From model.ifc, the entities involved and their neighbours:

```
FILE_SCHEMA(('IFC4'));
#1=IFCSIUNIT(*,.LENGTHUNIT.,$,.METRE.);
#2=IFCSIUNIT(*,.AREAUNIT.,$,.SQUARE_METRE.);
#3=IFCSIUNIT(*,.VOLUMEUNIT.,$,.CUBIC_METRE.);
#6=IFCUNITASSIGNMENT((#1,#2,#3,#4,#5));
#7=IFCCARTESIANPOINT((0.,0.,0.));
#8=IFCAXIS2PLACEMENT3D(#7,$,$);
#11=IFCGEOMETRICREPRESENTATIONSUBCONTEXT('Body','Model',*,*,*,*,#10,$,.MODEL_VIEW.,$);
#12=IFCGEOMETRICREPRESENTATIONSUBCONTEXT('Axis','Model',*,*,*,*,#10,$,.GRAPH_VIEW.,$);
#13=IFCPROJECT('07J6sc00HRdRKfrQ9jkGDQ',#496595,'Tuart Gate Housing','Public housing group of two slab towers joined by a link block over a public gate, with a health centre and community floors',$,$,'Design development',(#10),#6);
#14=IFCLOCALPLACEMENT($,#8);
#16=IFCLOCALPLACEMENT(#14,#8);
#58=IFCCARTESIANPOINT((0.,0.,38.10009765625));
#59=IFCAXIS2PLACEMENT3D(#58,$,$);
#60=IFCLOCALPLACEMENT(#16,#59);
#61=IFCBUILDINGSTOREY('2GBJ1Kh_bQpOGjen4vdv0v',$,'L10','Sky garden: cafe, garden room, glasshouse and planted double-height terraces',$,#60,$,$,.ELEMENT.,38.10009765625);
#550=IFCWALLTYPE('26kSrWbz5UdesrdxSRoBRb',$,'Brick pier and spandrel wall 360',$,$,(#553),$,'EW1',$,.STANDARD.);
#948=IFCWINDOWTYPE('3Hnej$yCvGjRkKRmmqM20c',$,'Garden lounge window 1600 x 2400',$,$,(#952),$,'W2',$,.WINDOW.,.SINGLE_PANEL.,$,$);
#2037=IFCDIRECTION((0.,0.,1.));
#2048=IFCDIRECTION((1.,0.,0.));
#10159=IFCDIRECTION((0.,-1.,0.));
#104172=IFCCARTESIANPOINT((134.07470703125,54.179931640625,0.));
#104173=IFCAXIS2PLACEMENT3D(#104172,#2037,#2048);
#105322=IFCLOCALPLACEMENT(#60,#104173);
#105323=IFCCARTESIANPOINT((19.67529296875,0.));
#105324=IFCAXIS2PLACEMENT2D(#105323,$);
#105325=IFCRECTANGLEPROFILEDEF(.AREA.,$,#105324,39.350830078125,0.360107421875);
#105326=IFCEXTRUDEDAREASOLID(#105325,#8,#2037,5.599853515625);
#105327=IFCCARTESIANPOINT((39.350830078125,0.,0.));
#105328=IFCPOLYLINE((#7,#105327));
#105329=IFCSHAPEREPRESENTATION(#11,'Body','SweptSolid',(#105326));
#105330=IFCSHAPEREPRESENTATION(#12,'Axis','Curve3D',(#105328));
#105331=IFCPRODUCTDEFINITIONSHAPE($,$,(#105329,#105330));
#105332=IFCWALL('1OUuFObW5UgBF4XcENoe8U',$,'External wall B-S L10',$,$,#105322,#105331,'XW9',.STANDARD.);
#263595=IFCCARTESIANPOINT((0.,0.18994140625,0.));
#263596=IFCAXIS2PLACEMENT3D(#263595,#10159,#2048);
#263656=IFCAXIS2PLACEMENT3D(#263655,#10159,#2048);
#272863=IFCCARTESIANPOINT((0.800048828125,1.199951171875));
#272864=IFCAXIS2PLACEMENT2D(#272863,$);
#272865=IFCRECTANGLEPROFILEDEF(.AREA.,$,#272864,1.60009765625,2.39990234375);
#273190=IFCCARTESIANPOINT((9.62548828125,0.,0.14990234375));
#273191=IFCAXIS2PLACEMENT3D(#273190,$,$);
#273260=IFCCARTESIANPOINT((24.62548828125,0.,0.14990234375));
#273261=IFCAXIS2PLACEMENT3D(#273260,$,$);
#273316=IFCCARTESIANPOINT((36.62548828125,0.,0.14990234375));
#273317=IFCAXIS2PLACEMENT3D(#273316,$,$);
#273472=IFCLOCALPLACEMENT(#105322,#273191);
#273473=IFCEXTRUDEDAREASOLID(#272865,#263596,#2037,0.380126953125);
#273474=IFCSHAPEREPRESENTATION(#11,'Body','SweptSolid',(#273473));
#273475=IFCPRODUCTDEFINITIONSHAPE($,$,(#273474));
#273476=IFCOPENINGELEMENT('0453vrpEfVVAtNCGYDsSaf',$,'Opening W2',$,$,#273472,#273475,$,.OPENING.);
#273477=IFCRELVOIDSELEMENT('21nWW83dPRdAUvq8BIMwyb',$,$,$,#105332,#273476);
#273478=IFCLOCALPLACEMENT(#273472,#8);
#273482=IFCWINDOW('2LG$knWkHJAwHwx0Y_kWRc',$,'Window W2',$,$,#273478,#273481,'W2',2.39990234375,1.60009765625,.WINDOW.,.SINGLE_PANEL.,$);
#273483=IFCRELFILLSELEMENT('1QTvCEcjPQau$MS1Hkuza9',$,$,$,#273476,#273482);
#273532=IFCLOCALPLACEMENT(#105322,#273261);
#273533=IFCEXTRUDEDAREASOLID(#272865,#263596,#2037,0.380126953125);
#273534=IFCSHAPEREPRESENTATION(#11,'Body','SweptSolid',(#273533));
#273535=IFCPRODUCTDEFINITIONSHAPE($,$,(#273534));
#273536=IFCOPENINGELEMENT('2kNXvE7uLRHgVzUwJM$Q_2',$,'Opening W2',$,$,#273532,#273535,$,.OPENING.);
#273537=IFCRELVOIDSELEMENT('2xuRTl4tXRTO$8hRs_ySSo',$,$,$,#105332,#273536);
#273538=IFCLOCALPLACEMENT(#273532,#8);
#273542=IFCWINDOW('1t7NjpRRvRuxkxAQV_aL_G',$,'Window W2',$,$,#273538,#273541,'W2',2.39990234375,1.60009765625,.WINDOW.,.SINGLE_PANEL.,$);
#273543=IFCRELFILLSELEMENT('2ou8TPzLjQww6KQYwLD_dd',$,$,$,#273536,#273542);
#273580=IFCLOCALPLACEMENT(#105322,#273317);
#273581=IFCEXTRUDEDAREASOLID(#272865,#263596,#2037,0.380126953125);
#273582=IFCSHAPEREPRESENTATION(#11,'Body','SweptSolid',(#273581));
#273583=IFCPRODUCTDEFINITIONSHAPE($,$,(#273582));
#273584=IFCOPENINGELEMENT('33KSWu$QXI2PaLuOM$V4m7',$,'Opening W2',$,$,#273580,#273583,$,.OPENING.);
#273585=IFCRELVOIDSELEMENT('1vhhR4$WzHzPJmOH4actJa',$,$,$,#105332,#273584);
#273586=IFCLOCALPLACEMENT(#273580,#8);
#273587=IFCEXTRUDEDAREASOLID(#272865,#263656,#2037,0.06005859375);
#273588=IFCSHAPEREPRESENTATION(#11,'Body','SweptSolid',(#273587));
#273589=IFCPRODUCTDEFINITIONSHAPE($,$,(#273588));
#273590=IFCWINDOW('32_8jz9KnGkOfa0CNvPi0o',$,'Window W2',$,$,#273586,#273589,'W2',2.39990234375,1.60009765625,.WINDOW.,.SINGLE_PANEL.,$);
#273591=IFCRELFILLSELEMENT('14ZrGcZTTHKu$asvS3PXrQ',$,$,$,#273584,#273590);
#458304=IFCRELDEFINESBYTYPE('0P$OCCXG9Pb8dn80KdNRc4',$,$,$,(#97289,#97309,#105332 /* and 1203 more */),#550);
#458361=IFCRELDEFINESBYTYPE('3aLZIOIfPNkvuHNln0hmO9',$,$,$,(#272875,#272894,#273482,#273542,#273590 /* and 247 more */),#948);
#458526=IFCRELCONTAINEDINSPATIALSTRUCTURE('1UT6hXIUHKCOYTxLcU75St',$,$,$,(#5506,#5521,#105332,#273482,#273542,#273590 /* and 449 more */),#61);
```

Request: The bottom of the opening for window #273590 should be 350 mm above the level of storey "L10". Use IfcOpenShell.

```python
import numpy as np
import ifcopenshell
import ifcopenshell.api.geometry
import ifcopenshell.geom
import ifcopenshell.util.element
import ifcopenshell.util.placement
import ifcopenshell.util.shape
import ifcopenshell.util.unit

model = ifcopenshell.open("model.ifc")
unit_scale = ifcopenshell.util.unit.calculate_unit_scale(model)

window = model.by_guid("32_8jz9KnGkOfa0CNvPi0o")
opening = window.FillsVoids[0].RelatingOpeningElement
storey = ifcopenshell.util.element.get_container(window, ifc_class="IfcBuildingStorey")
level = ifcopenshell.util.placement.get_local_placement(storey.ObjectPlacement)[2, 3]

# The opening's origin need not be at the sill, so measure its lowest point.
shape = ifcopenshell.geom.create_shape(ifcopenshell.geom.settings(), opening)
bottom = ifcopenshell.util.shape.get_shape_bottom_elevation(shape, shape.geometry) / unit_scale
dz = level + 0.35 - bottom

shift = np.array([0.0, 0.0, dz])
# The window is placed relative to its opening, so it follows when the opening moves.
matrix = ifcopenshell.util.placement.get_local_placement(opening.ObjectPlacement)
matrix[:3, 3] += shift
ifcopenshell.api.geometry.edit_object_placement(
    model, product=opening, matrix=matrix, is_si=False, should_transform_children=True
)

print(f"moved by {dz * unit_scale:+.3f} m")

model.write("model_updated.ifc")
```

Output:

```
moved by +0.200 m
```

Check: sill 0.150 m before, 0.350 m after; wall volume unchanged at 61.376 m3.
